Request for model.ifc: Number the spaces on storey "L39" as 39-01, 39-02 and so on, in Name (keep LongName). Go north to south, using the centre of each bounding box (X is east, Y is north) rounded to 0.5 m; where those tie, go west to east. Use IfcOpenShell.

First a look at what the model holds.

```python
import ifcopenshell
import ifcopenshell.util.element
import ifcopenshell.util.placement

model = ifcopenshell.open("model.ifc")
print(model.schema)
storey = next(s for s in model.by_type("IfcBuildingStorey") if s.Name == "L39")
spaces = [e for e in ifcopenshell.util.element.get_decomposition(storey) if e.is_a("IfcSpace")]
for e in sorted(spaces, key=lambda e: e.id()):
    origin = ifcopenshell.util.placement.get_local_placement(e.ObjectPlacement)[:3, 3]
    print(e.id(), e.Name, e.LongName, origin.round(2) + 0.0, sep=" | ")
```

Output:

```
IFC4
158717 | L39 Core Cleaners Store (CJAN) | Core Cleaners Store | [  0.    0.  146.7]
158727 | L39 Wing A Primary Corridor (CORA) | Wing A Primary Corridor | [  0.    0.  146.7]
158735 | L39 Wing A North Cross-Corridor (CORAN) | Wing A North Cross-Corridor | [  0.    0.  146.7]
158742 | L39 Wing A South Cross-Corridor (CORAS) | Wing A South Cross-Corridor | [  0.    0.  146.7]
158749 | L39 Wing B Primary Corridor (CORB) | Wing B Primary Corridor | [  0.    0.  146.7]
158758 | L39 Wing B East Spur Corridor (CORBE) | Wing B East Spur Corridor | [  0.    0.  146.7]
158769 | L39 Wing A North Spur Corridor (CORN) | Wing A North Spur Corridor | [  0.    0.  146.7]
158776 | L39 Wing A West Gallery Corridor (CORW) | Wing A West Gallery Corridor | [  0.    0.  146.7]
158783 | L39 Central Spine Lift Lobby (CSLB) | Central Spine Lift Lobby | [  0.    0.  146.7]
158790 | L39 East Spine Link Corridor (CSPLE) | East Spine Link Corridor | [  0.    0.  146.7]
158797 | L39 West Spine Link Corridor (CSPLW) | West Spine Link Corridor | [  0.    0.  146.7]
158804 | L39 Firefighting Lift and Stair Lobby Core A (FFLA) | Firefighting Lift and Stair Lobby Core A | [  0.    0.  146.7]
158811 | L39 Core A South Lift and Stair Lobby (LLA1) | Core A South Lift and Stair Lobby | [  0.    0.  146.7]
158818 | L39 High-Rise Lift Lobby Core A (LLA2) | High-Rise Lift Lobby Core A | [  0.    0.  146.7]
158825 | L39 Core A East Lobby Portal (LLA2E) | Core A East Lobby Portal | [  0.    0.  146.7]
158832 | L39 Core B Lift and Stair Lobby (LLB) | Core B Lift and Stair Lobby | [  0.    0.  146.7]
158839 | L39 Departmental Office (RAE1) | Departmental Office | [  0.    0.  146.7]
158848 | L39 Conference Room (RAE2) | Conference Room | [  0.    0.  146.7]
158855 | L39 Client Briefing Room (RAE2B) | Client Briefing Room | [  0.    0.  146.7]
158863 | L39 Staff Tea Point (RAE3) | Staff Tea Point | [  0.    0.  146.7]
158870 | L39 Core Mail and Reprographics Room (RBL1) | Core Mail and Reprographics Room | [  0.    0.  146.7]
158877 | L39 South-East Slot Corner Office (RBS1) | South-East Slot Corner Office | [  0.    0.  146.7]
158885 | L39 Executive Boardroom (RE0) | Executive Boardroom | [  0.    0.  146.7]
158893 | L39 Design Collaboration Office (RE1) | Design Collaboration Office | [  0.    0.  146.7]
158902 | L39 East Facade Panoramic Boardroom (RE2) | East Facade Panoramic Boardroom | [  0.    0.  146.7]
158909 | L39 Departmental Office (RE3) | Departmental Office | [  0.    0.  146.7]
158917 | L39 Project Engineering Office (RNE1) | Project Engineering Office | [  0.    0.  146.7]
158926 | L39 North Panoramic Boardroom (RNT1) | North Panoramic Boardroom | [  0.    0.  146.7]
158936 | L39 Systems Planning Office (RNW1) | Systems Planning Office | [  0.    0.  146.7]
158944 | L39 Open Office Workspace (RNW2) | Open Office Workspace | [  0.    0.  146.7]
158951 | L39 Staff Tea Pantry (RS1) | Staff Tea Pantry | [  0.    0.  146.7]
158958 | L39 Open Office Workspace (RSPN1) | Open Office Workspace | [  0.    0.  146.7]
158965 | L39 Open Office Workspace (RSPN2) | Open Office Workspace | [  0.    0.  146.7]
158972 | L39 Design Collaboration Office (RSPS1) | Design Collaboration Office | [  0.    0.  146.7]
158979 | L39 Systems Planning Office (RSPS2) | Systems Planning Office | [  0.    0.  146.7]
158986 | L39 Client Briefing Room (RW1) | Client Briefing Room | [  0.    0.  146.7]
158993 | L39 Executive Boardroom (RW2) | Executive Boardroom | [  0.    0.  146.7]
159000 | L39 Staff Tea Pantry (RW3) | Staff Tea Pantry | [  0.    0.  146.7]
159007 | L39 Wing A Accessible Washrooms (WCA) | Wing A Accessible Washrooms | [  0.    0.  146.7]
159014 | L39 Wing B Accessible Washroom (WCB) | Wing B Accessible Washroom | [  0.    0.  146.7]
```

```python
import ifcopenshell
import ifcopenshell.geom
import ifcopenshell.util.element
import ifcopenshell.util.shape

model = ifcopenshell.open("model.ifc")
settings = ifcopenshell.geom.settings()
settings.set("use-world-coords", True)


def centre(element):
    shape = ifcopenshell.geom.create_shape(settings, element)
    return ifcopenshell.util.shape.get_bbox_centroid(shape.geometry)


storey = next(s for s in model.by_type("IfcBuildingStorey") if s.Name == "L39")
spaces = [e for e in ifcopenshell.util.element.get_decomposition(storey) if e.is_a("IfcSpace")]

# Insertion points can sit at a corner or the storey origin, so sort by the geometry (in metres).
centres = {e: centre(e) for e in spaces}
spaces.sort(key=lambda e: (-round(centres[e][1] / 0.5), centres[e][0]))

for i, e in enumerate(spaces, start=1):
    number = f"39-{i:02d}"
    e.Name = number
    print(e.id(), number)

model.write("model_rev.ifc")
```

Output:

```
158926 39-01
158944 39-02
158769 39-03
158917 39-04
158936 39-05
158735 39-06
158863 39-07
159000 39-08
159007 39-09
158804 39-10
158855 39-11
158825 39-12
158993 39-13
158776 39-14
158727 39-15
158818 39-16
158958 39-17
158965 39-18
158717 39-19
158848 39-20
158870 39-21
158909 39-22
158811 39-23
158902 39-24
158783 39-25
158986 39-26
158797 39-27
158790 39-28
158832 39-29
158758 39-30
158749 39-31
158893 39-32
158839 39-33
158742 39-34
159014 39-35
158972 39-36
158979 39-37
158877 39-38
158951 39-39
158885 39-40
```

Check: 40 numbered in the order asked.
